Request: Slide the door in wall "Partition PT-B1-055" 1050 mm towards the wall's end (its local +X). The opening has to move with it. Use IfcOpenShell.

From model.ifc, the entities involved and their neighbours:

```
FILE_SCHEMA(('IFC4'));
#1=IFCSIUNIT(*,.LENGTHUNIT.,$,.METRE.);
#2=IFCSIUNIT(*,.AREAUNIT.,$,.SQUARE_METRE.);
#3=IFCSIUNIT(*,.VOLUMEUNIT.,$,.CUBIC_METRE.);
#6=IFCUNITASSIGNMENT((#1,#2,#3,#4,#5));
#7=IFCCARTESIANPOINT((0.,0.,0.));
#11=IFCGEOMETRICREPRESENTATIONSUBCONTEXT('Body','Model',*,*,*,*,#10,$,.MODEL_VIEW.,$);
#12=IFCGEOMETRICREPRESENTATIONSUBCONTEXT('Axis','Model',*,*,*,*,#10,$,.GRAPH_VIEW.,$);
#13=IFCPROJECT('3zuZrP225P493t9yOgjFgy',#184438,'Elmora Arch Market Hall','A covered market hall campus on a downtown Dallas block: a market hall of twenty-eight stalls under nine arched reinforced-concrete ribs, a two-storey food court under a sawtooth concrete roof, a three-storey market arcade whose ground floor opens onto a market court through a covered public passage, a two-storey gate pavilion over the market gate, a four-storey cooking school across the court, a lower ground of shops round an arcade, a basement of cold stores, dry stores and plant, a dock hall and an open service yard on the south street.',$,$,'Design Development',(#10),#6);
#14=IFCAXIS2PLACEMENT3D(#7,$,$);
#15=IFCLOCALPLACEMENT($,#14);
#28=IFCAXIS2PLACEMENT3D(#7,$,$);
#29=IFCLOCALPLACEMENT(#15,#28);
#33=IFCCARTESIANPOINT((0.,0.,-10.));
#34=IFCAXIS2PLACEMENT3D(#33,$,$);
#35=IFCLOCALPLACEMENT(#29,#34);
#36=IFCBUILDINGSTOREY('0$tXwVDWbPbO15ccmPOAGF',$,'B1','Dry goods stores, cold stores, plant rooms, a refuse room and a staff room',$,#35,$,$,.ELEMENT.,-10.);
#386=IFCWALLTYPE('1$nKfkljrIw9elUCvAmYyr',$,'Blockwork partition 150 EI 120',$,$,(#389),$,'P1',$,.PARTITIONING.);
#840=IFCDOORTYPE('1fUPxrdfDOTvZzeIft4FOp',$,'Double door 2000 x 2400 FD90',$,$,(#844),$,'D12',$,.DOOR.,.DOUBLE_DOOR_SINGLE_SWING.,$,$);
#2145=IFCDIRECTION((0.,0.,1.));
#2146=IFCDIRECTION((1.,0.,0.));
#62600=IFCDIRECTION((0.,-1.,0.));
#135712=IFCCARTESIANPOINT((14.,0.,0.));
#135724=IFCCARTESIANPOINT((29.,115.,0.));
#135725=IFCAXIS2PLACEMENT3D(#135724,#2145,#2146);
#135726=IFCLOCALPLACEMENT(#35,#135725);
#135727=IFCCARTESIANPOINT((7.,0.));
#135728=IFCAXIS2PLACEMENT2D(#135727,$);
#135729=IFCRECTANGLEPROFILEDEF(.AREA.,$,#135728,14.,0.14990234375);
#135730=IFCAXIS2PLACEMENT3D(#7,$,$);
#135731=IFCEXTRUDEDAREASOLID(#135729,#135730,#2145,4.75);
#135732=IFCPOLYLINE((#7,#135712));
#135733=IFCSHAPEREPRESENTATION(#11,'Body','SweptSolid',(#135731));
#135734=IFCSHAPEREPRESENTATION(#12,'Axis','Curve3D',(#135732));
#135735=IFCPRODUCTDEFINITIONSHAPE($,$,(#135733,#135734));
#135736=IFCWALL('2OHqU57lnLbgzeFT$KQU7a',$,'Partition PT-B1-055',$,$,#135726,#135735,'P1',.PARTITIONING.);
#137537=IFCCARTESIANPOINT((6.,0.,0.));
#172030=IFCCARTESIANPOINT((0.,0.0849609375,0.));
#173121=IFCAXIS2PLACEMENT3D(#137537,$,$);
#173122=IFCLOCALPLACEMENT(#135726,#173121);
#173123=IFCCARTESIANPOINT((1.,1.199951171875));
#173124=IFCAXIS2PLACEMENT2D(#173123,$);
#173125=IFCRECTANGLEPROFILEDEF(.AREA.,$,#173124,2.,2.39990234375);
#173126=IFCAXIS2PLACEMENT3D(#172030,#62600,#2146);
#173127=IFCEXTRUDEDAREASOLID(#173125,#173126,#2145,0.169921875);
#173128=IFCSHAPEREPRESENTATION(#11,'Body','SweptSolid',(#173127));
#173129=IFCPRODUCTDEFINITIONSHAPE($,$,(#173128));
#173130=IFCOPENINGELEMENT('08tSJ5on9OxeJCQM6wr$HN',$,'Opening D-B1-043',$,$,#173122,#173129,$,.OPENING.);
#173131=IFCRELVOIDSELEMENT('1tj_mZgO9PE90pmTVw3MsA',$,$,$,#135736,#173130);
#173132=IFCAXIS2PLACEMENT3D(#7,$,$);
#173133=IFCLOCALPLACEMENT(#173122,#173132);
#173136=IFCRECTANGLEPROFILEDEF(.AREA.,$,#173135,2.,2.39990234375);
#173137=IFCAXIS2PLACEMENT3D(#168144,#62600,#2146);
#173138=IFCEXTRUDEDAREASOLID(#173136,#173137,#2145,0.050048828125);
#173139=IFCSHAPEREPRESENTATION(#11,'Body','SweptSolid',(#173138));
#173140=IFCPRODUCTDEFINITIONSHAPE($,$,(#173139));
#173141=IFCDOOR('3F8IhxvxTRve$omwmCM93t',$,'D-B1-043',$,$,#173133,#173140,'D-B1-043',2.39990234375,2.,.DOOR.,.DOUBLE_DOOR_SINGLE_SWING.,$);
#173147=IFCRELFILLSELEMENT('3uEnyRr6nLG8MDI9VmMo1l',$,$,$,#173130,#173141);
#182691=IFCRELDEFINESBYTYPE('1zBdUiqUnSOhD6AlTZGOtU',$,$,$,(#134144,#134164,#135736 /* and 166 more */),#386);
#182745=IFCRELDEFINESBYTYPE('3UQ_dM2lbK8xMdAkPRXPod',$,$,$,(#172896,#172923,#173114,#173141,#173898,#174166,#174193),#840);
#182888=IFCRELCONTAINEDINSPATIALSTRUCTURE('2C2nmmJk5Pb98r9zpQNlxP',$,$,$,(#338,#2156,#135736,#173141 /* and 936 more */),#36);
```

```python
import ifcopenshell
import ifcopenshell.api.geometry
import ifcopenshell.util.placement
import ifcopenshell.util.unit

model = ifcopenshell.open("model.ifc")
unit_scale = ifcopenshell.util.unit.calculate_unit_scale(model)

door = model.by_guid("3F8IhxvxTRve$omwmCM93t")
opening = door.FillsVoids[0].RelatingOpeningElement
wall = opening.VoidsElements[0].RelatingBuildingElement

wall_matrix = ifcopenshell.util.placement.get_local_placement(wall.ObjectPlacement)
shift = wall_matrix[:3, 0] * 1.05 / unit_scale
before = ifcopenshell.util.placement.get_local_placement(door.ObjectPlacement)[:3, 3].copy()

# The door is placed relative to its opening, so it follows when the opening moves.
matrix = ifcopenshell.util.placement.get_local_placement(opening.ObjectPlacement)
matrix[:3, 3] += shift
ifcopenshell.api.geometry.edit_object_placement(
    model, product=opening, matrix=matrix, is_si=False, should_transform_children=True
)

after = ifcopenshell.util.placement.get_local_placement(door.ObjectPlacement)[:3, 3]
print("door moved by", (after - before).round(3) + 0.0)

model.write("model-out.ifc")
```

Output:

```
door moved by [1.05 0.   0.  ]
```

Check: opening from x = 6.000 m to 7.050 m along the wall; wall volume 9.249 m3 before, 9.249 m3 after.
